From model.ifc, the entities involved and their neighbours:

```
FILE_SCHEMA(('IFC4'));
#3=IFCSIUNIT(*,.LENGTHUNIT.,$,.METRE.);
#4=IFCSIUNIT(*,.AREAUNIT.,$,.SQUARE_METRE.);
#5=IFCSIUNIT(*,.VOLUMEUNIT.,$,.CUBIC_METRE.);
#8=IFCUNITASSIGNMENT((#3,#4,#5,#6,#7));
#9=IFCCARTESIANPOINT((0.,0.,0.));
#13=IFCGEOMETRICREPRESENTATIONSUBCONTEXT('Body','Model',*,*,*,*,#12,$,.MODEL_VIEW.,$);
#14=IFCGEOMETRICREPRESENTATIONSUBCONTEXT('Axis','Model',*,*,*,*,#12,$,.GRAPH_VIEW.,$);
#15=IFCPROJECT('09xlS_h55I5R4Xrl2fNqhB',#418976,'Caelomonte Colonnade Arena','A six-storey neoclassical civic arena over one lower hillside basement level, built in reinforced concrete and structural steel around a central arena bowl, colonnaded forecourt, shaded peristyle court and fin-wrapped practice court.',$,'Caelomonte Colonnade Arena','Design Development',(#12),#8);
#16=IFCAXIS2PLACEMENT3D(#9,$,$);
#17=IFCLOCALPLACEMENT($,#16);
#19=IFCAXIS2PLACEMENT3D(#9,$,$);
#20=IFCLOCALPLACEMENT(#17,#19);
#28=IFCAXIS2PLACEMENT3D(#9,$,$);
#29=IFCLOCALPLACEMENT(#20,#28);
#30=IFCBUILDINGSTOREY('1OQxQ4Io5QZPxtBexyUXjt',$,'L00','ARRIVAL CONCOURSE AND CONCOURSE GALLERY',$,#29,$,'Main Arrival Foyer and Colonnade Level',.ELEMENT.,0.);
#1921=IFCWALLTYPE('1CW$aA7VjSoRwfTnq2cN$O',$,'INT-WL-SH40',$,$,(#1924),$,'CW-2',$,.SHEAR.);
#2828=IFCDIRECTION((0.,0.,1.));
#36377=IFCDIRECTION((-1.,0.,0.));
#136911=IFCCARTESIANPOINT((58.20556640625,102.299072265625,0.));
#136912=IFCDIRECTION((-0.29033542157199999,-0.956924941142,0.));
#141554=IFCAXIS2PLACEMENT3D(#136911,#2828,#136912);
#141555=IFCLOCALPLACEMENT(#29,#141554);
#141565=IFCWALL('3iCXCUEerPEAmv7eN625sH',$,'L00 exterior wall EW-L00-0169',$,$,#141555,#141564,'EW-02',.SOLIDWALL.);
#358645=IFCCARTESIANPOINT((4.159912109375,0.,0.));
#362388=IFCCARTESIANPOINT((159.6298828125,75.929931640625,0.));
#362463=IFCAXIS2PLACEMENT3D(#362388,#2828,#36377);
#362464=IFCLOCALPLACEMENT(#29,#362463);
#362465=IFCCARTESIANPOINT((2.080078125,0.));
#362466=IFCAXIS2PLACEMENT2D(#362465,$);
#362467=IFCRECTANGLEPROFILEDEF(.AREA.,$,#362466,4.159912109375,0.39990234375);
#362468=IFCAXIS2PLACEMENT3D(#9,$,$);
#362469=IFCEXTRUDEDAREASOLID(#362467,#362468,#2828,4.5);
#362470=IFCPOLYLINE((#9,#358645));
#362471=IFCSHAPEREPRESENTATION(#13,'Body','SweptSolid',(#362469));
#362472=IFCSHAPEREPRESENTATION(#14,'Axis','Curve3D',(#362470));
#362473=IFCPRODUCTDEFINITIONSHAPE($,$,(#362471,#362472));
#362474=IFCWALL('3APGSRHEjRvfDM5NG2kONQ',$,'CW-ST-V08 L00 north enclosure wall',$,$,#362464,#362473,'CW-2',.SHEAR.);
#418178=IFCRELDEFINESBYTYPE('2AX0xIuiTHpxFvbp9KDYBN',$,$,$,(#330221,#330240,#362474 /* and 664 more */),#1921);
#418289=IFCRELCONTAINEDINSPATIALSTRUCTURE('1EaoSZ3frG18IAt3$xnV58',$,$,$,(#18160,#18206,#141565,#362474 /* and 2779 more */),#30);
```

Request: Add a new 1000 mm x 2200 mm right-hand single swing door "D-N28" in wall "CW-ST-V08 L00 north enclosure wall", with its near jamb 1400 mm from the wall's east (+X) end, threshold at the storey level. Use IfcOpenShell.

```python
import numpy as np
import ifcopenshell
import ifcopenshell.api.feature
import ifcopenshell.api.geometry
import ifcopenshell.api.root
import ifcopenshell.api.spatial
import ifcopenshell.geom
import ifcopenshell.util.element
import ifcopenshell.util.placement
import ifcopenshell.util.representation
import ifcopenshell.util.shape
import ifcopenshell.util.unit

model = ifcopenshell.open("model.ifc")
unit_scale = ifcopenshell.util.unit.calculate_unit_scale(model)
settings = ifcopenshell.geom.settings()


def volume(element):
    """Net volume in cubic metres, openings subtracted."""
    shape = ifcopenshell.geom.create_shape(settings, element)
    return ifcopenshell.util.shape.get_volume(shape.geometry)


wall = model.by_id(362474)
storey = ifcopenshell.util.element.get_container(wall, ifc_class="IfcBuildingStorey")
context = ifcopenshell.util.representation.get_context(model, "Model", "Body", "MODEL_VIEW")
before = volume(wall)

width, height, from_end, sill = 1, 2.2, 1.4, 0.0  # metres

# The wall runs along its own X axis, and the end named is its -X end.
wall_shape = ifcopenshell.geom.create_shape(settings, wall)
x, y, z = ifcopenshell.util.shape.get_vertices(wall_shape.geometry).T
start = x.min() + from_end
face, thickness = float(y.min()), float(y.max() - y.min())
wall_matrix = ifcopenshell.util.placement.get_local_placement(wall.ObjectPlacement)
level = ifcopenshell.util.placement.get_local_placement(storey.ObjectPlacement)[2, 3]


def in_wall(x, y):
    """Placement at x, y metres in the wall's axes, at sill height."""
    matrix = wall_matrix.copy()
    matrix[:, 3] = wall_matrix @ np.array([x / unit_scale, y / unit_scale, 0.0, 1.0])
    matrix[2, 3] = level + sill / unit_scale
    return matrix


# Opening: a box that overshoots both wall faces by 50 mm.
opening = ifcopenshell.api.root.create_entity(model, ifc_class="IfcOpeningElement", predefined_type="OPENING")
box = ifcopenshell.api.geometry.add_wall_representation(
    model, context=context, length=width, height=height, thickness=thickness + 0.1
)
ifcopenshell.api.geometry.assign_representation(model, product=opening, representation=box)
ifcopenshell.api.geometry.edit_object_placement(model, product=opening, matrix=in_wall(start, face - 0.05), is_si=False)
ifcopenshell.api.feature.add_feature(model, feature=opening, element=wall)

door = ifcopenshell.api.root.create_entity(model, ifc_class="IfcDoor", name="D-N28", predefined_type="DOOR")
door.OverallWidth, door.OverallHeight = width / unit_scale, height / unit_scale
door.OperationType = "SINGLE_SWING_RIGHT"
body = ifcopenshell.api.geometry.add_door_representation(
    model,
    context=context,
    overall_width=door.OverallWidth,
    overall_height=door.OverallHeight,
    operation_type="SINGLE_SWING_RIGHT",
    lining_properties={"LiningDepth": thickness / unit_scale, "ThresholdDepth": thickness / unit_scale},
)
ifcopenshell.api.geometry.assign_representation(model, product=door, representation=body)
ifcopenshell.api.spatial.assign_container(model, products=[door], relating_structure=storey)
ifcopenshell.api.feature.add_filling(model, opening=opening, element=door)

# The lining spans the wall, so the door starts at the wall face.
ifcopenshell.api.geometry.edit_object_placement(model, product=door, matrix=in_wall(start, face), is_si=False)

after = volume(wall)

print(f"wall volume {before:.3f} -> {after:.3f} m3")

model.write("model_edited.ifc")
```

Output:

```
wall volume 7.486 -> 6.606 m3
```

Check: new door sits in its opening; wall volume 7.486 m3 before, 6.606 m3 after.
